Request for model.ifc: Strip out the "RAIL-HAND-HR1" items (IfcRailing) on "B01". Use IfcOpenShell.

First a look at what the model holds.

```python
import ifcopenshell
import ifcopenshell.util.element

model = ifcopenshell.open("model.ifc")
print(model.schema)
storey = next(s for s in model.by_type("IfcBuildingStorey") if s.Name == "B01")
railings = [e for e in ifcopenshell.util.element.get_decomposition(storey) if e.is_a("IfcRailing")]
seen = {}
for e in railings:
    element_type = ifcopenshell.util.element.get_type(e)
    name = element_type.Name if element_type not in (None, e) else None
    seen[name] = seen.get(name, 0) + 1
for name, count in sorted(seen.items(), key=str):
    print(count, "x", name)
```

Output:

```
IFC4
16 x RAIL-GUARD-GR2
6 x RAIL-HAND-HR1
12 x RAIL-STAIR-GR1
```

```python
import ifcopenshell
import ifcopenshell.api.root
import ifcopenshell.util.element

model = ifcopenshell.open("model.ifc")

storey = next(s for s in model.by_type("IfcBuildingStorey") if s.Name == "B01")
railings = [e for e in ifcopenshell.util.element.get_decomposition(storey) if e.is_a("IfcRailing")]
targets = [e for e in railings if (t := ifcopenshell.util.element.get_type(e)) not in (None, e) and t.Name == "RAIL-HAND-HR1"]

for e in targets:
    ifcopenshell.api.root.remove_product(model, product=e)
print(len(targets), "removed")

model.write("model_v2.ifc")
```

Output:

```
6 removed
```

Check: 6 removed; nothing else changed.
